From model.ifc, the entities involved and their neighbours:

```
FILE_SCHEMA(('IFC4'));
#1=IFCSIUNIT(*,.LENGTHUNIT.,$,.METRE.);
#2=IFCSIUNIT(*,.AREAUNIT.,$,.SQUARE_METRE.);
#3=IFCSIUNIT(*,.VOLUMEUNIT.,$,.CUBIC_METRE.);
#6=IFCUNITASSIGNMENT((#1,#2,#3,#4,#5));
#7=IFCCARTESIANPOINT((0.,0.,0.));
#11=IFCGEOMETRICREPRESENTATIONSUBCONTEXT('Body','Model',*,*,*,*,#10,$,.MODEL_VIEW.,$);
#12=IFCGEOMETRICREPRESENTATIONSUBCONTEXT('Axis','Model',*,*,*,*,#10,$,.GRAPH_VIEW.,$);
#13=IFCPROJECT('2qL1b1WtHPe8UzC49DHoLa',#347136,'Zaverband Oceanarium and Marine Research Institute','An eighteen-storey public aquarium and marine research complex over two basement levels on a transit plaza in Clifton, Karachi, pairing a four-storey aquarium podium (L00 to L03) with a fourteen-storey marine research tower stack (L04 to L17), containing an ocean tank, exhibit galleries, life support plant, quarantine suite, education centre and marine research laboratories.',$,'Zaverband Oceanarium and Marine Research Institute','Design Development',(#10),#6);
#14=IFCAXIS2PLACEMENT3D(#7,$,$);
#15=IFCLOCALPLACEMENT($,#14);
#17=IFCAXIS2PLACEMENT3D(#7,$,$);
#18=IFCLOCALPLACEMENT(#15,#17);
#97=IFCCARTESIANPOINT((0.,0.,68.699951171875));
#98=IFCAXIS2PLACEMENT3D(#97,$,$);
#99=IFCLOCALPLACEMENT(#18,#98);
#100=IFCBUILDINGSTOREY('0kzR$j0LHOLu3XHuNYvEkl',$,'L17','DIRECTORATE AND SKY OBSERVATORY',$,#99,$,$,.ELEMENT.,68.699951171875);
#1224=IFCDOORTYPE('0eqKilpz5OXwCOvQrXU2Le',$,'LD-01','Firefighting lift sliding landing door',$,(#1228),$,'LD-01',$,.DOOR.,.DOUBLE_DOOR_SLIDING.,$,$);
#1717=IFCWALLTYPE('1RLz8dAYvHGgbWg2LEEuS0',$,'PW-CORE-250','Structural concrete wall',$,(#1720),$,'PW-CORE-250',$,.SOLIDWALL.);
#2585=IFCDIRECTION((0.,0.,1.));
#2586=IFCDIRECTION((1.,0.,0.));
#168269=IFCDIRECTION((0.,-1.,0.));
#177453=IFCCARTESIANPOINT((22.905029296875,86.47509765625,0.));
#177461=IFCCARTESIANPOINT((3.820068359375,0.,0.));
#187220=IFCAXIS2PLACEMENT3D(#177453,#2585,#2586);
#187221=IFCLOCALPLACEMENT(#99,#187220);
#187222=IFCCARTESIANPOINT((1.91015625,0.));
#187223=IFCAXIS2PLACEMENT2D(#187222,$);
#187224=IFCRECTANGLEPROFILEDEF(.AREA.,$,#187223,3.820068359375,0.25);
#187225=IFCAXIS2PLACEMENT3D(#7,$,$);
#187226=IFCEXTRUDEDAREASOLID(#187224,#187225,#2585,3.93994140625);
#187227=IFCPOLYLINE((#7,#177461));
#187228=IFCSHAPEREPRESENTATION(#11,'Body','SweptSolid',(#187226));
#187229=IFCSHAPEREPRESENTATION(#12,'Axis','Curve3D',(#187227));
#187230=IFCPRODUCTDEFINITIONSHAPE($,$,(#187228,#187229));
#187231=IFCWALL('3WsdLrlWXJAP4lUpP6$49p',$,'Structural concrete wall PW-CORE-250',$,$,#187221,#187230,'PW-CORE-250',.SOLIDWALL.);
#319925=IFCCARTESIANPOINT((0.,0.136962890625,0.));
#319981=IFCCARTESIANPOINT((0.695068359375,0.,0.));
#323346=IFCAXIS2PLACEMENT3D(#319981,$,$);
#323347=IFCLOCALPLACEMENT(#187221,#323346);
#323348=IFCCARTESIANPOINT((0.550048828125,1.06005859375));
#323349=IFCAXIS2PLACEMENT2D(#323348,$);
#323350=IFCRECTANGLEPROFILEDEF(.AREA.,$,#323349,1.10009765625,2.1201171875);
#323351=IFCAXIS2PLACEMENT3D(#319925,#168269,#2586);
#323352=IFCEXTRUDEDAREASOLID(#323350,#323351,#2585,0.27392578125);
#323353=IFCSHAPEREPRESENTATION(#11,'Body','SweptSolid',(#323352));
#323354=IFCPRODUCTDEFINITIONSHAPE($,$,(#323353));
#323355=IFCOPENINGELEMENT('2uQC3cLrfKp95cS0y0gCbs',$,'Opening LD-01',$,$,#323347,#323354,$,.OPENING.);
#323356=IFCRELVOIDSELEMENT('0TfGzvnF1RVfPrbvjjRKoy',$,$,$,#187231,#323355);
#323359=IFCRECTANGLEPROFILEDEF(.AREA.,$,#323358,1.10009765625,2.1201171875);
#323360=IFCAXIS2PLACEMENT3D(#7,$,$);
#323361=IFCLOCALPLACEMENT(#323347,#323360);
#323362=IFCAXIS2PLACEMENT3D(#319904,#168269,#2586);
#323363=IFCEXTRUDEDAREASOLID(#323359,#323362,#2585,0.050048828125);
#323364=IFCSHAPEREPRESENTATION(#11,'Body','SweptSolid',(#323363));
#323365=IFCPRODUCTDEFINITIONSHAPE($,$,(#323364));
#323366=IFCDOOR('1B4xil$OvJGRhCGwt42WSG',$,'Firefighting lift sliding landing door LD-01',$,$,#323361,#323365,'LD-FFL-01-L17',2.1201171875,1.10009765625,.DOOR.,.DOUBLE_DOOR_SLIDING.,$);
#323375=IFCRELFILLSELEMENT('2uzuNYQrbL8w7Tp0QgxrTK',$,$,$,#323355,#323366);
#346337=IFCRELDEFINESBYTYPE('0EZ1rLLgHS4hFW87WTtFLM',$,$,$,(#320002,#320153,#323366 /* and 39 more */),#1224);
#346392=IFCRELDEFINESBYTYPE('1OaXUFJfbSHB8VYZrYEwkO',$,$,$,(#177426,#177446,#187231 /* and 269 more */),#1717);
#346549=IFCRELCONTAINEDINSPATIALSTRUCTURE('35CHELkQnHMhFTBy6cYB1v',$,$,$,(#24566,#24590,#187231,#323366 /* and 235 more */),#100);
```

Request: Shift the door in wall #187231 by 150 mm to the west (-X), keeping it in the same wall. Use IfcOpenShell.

```python
import ifcopenshell
import ifcopenshell.api.geometry
import ifcopenshell.util.placement
import ifcopenshell.util.unit

model = ifcopenshell.open("model.ifc")
unit_scale = ifcopenshell.util.unit.calculate_unit_scale(model)

door = model.by_guid("1B4xil$OvJGRhCGwt42WSG")
opening = door.FillsVoids[0].RelatingOpeningElement
wall = opening.VoidsElements[0].RelatingBuildingElement

wall_matrix = ifcopenshell.util.placement.get_local_placement(wall.ObjectPlacement)
shift = wall_matrix[:3, 0] * -0.15 / unit_scale
before = ifcopenshell.util.placement.get_local_placement(door.ObjectPlacement)[:3, 3].copy()

# The door is placed relative to its opening, so it follows when the opening moves.
matrix = ifcopenshell.util.placement.get_local_placement(opening.ObjectPlacement)
matrix[:3, 3] += shift
ifcopenshell.api.geometry.edit_object_placement(
    model, product=opening, matrix=matrix, is_si=False, should_transform_children=True
)

after = ifcopenshell.util.placement.get_local_placement(door.ObjectPlacement)[:3, 3]
print("door moved by", (after - before).round(3) + 0.0)

model.write("model_edited.ifc")
```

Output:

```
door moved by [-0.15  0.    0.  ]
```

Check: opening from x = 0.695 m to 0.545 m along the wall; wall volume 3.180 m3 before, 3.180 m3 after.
